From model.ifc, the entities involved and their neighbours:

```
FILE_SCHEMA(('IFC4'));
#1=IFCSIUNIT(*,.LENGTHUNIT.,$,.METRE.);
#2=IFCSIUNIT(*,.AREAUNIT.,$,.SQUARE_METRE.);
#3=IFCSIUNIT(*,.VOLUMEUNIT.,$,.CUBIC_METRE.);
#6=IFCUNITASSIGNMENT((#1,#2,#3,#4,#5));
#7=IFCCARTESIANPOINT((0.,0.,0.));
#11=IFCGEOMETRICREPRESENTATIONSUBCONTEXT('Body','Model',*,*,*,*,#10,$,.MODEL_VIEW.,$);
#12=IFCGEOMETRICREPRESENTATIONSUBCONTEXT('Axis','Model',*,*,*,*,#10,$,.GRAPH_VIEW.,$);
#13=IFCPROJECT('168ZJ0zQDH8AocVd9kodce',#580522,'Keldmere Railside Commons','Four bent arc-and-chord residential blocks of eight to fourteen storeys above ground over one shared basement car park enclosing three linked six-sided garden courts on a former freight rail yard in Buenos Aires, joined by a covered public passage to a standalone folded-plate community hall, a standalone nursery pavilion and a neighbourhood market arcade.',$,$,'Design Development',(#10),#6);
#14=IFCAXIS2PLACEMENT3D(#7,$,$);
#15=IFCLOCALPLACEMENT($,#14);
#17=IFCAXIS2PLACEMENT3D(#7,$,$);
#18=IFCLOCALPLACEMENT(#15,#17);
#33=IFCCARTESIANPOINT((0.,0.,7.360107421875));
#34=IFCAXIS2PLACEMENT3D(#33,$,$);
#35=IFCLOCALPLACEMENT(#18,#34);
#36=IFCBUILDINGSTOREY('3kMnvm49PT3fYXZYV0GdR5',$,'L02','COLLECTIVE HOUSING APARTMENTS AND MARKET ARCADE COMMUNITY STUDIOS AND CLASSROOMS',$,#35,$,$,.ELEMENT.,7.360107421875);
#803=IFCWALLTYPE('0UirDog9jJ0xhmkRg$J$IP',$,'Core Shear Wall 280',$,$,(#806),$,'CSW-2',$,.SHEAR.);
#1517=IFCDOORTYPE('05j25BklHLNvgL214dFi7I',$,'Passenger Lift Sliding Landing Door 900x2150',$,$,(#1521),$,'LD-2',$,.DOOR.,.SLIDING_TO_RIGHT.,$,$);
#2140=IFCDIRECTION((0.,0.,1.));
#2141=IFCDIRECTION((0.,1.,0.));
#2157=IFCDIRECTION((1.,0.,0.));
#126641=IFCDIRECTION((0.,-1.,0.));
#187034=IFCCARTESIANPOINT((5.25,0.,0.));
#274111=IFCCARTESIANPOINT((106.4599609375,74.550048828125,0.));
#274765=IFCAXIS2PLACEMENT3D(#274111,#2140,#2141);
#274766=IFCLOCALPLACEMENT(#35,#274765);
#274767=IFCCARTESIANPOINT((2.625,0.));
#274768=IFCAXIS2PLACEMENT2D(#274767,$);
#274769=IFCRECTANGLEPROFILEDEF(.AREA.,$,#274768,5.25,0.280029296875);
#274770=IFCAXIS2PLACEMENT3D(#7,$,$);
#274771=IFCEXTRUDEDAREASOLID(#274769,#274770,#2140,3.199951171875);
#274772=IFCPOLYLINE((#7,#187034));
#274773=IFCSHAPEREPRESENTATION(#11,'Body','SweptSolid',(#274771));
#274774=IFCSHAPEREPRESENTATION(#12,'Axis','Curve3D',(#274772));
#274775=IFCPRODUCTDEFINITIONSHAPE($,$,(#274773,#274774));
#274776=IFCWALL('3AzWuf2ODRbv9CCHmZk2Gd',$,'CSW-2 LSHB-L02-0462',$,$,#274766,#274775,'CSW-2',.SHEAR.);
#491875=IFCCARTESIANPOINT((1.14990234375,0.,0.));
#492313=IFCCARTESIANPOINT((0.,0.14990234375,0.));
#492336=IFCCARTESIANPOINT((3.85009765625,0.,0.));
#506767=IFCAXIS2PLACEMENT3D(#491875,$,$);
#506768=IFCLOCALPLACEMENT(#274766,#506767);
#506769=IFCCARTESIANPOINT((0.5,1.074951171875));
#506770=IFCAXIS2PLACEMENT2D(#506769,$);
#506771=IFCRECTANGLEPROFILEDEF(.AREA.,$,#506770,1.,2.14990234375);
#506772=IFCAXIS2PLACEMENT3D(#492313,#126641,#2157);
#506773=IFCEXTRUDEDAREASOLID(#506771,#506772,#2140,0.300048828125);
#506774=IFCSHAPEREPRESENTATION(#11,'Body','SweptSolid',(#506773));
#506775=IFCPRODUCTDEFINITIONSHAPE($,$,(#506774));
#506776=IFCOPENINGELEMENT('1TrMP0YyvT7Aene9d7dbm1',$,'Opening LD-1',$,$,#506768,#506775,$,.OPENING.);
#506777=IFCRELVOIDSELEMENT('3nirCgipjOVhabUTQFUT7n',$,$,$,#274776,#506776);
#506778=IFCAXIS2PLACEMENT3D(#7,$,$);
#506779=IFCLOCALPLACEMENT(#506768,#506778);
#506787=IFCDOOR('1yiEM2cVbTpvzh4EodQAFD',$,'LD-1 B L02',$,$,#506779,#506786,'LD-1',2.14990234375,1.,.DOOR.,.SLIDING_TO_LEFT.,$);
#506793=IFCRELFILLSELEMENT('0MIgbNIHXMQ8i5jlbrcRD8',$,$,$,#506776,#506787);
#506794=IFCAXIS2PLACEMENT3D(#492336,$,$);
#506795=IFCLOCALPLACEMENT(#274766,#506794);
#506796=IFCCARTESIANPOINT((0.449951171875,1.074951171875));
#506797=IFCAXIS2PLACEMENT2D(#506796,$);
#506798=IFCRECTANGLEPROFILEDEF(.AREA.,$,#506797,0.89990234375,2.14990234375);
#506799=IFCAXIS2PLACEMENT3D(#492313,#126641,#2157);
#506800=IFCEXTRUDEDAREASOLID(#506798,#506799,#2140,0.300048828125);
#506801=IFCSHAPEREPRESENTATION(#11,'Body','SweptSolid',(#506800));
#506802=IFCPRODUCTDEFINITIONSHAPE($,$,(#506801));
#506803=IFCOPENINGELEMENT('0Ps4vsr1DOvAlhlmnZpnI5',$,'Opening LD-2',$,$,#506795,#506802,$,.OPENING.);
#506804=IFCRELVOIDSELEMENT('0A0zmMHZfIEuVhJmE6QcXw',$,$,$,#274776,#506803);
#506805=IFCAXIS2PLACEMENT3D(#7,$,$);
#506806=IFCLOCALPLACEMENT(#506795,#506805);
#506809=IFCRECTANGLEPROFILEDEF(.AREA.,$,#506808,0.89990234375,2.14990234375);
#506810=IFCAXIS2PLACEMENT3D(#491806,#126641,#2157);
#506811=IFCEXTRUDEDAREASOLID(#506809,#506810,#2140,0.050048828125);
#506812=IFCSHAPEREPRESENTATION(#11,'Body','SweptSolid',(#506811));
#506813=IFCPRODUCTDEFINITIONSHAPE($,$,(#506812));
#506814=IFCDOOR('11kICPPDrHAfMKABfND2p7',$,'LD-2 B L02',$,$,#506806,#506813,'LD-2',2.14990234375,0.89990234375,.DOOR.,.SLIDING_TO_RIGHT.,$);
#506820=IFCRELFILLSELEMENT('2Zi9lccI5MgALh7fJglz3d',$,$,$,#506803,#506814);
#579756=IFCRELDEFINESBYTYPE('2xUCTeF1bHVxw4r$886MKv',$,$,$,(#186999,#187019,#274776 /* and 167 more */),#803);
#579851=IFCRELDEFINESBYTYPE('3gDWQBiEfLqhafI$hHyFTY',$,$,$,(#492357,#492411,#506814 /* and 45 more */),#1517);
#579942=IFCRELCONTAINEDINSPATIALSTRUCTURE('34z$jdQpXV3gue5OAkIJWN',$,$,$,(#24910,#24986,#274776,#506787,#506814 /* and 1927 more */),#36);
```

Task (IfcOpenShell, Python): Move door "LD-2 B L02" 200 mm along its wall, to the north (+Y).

```python
import ifcopenshell
import ifcopenshell.api.geometry
import ifcopenshell.util.placement
import ifcopenshell.util.unit

model = ifcopenshell.open("model.ifc")
unit_scale = ifcopenshell.util.unit.calculate_unit_scale(model)

door = model.by_guid("11kICPPDrHAfMKABfND2p7")
opening = door.FillsVoids[0].RelatingOpeningElement
wall = opening.VoidsElements[0].RelatingBuildingElement

wall_matrix = ifcopenshell.util.placement.get_local_placement(wall.ObjectPlacement)
shift = wall_matrix[:3, 0] * 0.2 / unit_scale
before = ifcopenshell.util.placement.get_local_placement(door.ObjectPlacement)[:3, 3].copy()

# The door is placed relative to its opening, so it follows when the opening moves.
matrix = ifcopenshell.util.placement.get_local_placement(opening.ObjectPlacement)
matrix[:3, 3] += shift
ifcopenshell.api.geometry.edit_object_placement(
    model, product=opening, matrix=matrix, is_si=False, should_transform_children=True
)

after = ifcopenshell.util.placement.get_local_placement(door.ObjectPlacement)[:3, 3]
print("door moved by", (after - before).round(3) + 0.0)

model.write("model_v2.ifc")
```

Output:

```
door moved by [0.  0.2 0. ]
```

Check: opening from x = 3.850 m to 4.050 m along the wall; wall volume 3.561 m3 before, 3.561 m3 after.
